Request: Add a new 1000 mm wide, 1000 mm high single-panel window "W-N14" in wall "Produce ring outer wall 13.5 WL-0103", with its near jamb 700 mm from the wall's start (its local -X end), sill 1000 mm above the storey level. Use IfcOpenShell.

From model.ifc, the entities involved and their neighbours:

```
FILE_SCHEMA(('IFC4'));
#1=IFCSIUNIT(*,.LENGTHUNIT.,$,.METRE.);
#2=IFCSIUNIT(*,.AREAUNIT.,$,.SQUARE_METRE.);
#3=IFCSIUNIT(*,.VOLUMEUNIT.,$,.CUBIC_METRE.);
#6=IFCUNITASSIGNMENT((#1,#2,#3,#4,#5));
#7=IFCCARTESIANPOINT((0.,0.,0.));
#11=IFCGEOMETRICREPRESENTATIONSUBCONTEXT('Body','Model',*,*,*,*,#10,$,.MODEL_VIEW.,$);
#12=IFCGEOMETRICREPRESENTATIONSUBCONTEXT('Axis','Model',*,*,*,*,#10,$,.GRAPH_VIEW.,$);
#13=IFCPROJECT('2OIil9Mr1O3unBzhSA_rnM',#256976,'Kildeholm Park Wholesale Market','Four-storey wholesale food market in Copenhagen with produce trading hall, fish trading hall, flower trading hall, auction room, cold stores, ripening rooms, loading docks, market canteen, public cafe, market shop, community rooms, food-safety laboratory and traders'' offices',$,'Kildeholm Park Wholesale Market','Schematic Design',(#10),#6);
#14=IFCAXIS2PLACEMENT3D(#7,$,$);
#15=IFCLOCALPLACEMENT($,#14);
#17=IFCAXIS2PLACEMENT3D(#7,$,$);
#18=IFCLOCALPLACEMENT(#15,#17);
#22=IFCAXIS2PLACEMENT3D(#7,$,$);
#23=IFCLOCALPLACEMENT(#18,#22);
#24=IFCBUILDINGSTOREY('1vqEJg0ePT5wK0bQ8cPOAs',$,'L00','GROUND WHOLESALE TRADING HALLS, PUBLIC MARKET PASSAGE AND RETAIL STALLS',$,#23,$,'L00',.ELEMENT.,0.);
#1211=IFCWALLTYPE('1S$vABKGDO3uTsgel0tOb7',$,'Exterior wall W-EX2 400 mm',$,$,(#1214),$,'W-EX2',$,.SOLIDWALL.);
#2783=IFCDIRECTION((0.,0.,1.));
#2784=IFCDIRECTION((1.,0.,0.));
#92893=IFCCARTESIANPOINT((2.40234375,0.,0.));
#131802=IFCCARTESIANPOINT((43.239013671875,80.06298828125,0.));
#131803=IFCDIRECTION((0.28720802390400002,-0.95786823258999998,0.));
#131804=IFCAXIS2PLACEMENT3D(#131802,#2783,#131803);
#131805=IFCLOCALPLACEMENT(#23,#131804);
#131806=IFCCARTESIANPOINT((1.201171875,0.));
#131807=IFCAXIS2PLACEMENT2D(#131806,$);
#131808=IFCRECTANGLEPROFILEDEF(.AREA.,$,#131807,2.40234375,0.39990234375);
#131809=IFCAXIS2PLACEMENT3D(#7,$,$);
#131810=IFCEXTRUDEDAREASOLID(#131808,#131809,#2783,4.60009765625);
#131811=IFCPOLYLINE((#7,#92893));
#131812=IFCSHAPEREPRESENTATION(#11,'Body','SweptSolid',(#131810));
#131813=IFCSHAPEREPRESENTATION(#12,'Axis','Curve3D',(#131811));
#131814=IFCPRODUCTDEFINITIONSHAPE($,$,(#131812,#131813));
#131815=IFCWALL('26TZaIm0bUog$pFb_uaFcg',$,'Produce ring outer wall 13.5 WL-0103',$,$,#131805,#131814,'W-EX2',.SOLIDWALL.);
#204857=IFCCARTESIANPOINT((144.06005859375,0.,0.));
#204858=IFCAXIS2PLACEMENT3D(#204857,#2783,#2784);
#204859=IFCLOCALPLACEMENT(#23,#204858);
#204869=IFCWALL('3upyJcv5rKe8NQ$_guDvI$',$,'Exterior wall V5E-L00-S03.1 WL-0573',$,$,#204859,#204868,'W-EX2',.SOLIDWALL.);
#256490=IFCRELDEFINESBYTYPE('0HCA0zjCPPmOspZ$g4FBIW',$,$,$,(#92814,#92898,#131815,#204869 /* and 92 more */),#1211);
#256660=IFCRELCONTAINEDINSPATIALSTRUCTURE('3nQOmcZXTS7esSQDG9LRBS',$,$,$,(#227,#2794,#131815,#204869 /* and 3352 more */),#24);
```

```python
import numpy as np
import ifcopenshell
import ifcopenshell.api.feature
import ifcopenshell.api.geometry
import ifcopenshell.api.root
import ifcopenshell.api.spatial
import ifcopenshell.geom
import ifcopenshell.util.element
import ifcopenshell.util.placement
import ifcopenshell.util.representation
import ifcopenshell.util.shape
import ifcopenshell.util.unit

model = ifcopenshell.open("model.ifc")
unit_scale = ifcopenshell.util.unit.calculate_unit_scale(model)
settings = ifcopenshell.geom.settings()


def volume(element):
    """Net volume in cubic metres, openings subtracted."""
    shape = ifcopenshell.geom.create_shape(settings, element)
    return ifcopenshell.util.shape.get_volume(shape.geometry)


wall = model.by_guid("26TZaIm0bUog$pFb_uaFcg")
storey = ifcopenshell.util.element.get_container(wall, ifc_class="IfcBuildingStorey")
context = ifcopenshell.util.representation.get_context(model, "Model", "Body", "MODEL_VIEW")
before = volume(wall)

width, height, from_end, sill = 1, 1, 0.7, 1  # metres

# The wall runs along its own X axis, and the end named is its -X end.
wall_shape = ifcopenshell.geom.create_shape(settings, wall)
x, y, z = ifcopenshell.util.shape.get_vertices(wall_shape.geometry).T
start = x.min() + from_end
face, thickness = float(y.min()), float(y.max() - y.min())
wall_matrix = ifcopenshell.util.placement.get_local_placement(wall.ObjectPlacement)
level = ifcopenshell.util.placement.get_local_placement(storey.ObjectPlacement)[2, 3]


def in_wall(x, y):
    """Placement at x, y metres in the wall's axes, at sill height."""
    matrix = wall_matrix.copy()
    matrix[:, 3] = wall_matrix @ np.array([x / unit_scale, y / unit_scale, 0.0, 1.0])
    matrix[2, 3] = level + sill / unit_scale
    return matrix


# Opening: a box that overshoots both wall faces by 50 mm.
opening = ifcopenshell.api.root.create_entity(model, ifc_class="IfcOpeningElement", predefined_type="OPENING")
box = ifcopenshell.api.geometry.add_wall_representation(
    model, context=context, length=width, height=height, thickness=thickness + 0.1
)
ifcopenshell.api.geometry.assign_representation(model, product=opening, representation=box)
ifcopenshell.api.geometry.edit_object_placement(model, product=opening, matrix=in_wall(start, face - 0.05), is_si=False)
ifcopenshell.api.feature.add_feature(model, feature=opening, element=wall)

window = ifcopenshell.api.root.create_entity(model, ifc_class="IfcWindow", name="W-N14", predefined_type="WINDOW")
window.OverallWidth, window.OverallHeight = width / unit_scale, height / unit_scale
window.PartitioningType = "SINGLE_PANEL"
body = ifcopenshell.api.geometry.add_window_representation(
    model,
    context=context,
    overall_width=window.OverallWidth,
    overall_height=window.OverallHeight,
    partition_type="SINGLE_PANEL",
)
ifcopenshell.api.geometry.assign_representation(model, product=window, representation=body)
ifcopenshell.api.spatial.assign_container(model, products=[window], relating_structure=storey)
ifcopenshell.api.feature.add_filling(model, opening=opening, element=window)

# Centre the window in the wall's thickness.
ifcopenshell.api.geometry.edit_object_placement(model, product=window, matrix=in_wall(start, face), is_si=False)
window_shape = ifcopenshell.geom.create_shape(settings, window)
depth = ifcopenshell.util.shape.get_vertices(window_shape.geometry)[:, 1]
offset = face + thickness / 2 - (depth.min() + depth.max()) / 2
ifcopenshell.api.geometry.edit_object_placement(model, product=window, matrix=in_wall(start, offset), is_si=False)

after = volume(wall)

print(f"wall volume {before:.3f} -> {after:.3f} m3")

model.write("model-out.ifc")
```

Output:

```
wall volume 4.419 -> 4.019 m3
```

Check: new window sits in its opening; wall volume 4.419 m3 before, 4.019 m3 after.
